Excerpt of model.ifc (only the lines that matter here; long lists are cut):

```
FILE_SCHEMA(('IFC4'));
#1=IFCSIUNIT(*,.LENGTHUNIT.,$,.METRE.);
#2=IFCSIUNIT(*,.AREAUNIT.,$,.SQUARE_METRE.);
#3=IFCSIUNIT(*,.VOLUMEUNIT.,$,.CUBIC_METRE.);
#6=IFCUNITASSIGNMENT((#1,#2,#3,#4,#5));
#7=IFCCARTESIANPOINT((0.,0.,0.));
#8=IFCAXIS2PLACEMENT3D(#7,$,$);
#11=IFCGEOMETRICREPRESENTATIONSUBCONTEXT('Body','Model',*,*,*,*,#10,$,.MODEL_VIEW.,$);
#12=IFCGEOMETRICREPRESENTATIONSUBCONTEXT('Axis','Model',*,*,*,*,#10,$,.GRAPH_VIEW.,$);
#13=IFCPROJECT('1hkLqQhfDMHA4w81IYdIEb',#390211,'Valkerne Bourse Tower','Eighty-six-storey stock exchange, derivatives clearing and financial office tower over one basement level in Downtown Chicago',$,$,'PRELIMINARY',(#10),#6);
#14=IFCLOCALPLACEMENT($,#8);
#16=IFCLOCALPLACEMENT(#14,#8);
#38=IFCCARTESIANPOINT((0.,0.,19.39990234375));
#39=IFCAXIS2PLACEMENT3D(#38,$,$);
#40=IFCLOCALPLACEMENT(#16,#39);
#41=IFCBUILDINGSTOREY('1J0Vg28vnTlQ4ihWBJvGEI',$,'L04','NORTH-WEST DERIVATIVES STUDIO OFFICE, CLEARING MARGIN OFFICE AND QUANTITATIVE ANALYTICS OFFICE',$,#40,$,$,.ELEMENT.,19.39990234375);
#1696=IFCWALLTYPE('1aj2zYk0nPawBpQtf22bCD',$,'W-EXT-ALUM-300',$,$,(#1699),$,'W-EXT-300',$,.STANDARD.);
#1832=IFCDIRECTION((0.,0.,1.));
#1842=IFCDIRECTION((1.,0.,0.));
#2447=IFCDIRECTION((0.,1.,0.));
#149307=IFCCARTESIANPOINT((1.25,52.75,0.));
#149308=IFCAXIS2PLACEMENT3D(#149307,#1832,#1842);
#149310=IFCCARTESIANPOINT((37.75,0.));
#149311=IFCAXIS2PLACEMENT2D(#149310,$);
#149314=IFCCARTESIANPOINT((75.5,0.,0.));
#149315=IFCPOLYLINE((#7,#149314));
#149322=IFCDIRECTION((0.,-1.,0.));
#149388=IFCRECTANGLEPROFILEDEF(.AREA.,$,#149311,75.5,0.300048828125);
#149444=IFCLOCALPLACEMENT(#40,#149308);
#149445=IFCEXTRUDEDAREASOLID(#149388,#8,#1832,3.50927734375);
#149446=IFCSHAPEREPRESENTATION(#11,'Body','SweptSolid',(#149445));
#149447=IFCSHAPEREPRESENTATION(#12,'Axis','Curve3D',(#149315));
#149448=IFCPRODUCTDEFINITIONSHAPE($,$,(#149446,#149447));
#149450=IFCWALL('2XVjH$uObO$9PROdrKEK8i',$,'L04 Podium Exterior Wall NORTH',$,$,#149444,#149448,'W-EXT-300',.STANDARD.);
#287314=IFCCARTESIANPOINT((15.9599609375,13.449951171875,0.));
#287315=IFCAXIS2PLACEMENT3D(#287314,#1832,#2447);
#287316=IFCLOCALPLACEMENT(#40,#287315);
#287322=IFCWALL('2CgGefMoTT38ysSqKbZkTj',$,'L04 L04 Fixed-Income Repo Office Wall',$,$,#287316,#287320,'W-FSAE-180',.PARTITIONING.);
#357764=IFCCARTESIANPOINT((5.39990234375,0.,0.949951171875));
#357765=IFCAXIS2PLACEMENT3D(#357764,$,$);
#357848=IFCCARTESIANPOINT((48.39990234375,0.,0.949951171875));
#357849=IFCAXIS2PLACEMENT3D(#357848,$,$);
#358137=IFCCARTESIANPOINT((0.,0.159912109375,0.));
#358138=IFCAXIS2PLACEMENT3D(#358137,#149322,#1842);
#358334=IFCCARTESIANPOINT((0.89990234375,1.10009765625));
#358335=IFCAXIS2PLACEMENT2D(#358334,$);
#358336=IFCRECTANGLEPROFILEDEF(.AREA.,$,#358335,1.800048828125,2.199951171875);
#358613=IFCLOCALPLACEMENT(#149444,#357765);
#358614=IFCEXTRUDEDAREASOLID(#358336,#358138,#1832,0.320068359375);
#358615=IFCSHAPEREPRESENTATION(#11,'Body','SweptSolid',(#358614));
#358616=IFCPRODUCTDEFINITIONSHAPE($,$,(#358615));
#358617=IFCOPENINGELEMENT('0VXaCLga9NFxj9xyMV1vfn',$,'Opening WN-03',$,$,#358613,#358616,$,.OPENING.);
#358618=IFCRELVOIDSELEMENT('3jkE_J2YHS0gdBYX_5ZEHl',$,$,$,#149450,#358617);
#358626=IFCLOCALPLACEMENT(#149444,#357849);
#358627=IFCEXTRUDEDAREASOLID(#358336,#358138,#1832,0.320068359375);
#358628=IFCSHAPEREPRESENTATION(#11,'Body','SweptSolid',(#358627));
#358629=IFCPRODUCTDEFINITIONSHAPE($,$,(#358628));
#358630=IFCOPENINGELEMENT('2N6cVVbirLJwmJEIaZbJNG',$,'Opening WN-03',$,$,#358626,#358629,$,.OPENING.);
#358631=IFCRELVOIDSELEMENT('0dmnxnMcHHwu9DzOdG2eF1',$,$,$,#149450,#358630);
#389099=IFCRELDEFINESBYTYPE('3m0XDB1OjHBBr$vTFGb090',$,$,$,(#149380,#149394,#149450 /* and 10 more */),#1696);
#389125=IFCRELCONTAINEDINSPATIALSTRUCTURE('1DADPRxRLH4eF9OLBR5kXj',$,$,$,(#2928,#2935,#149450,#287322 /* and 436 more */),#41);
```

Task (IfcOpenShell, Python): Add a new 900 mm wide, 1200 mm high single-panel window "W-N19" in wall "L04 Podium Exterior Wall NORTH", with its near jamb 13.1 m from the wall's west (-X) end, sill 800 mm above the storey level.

```python
import numpy as np
import ifcopenshell
import ifcopenshell.api.feature
import ifcopenshell.api.geometry
import ifcopenshell.api.root
import ifcopenshell.api.spatial
import ifcopenshell.geom
import ifcopenshell.util.element
import ifcopenshell.util.placement
import ifcopenshell.util.representation
import ifcopenshell.util.shape
import ifcopenshell.util.unit

model = ifcopenshell.open("model.ifc")
unit_scale = ifcopenshell.util.unit.calculate_unit_scale(model)
settings = ifcopenshell.geom.settings()


def volume(element):
    """Net volume in cubic metres, openings subtracted."""
    shape = ifcopenshell.geom.create_shape(settings, element)
    return ifcopenshell.util.shape.get_volume(shape.geometry)


wall = model.by_id(149450)
storey = ifcopenshell.util.element.get_container(wall, ifc_class="IfcBuildingStorey")
context = ifcopenshell.util.representation.get_context(model, "Model", "Body", "MODEL_VIEW")
before = volume(wall)

width, height, from_end, sill = 0.9, 1.2, 13.1, 0.8  # metres

# The wall runs along its own X axis, and the end named is its -X end.
wall_shape = ifcopenshell.geom.create_shape(settings, wall)
x, y, z = ifcopenshell.util.shape.get_vertices(wall_shape.geometry).T
start = x.min() + from_end
face, thickness = float(y.min()), float(y.max() - y.min())
wall_matrix = ifcopenshell.util.placement.get_local_placement(wall.ObjectPlacement)
level = ifcopenshell.util.placement.get_local_placement(storey.ObjectPlacement)[2, 3]


def in_wall(x, y):
    """Placement at x, y metres in the wall's axes, at sill height."""
    matrix = wall_matrix.copy()
    matrix[:, 3] = wall_matrix @ np.array([x / unit_scale, y / unit_scale, 0.0, 1.0])
    matrix[2, 3] = level + sill / unit_scale
    return matrix


# Opening: a box that overshoots both wall faces by 50 mm.
opening = ifcopenshell.api.root.create_entity(model, ifc_class="IfcOpeningElement", predefined_type="OPENING")
box = ifcopenshell.api.geometry.add_wall_representation(
    model, context=context, length=width, height=height, thickness=thickness + 0.1
)
ifcopenshell.api.geometry.assign_representation(model, product=opening, representation=box)
ifcopenshell.api.geometry.edit_object_placement(model, product=opening, matrix=in_wall(start, face - 0.05), is_si=False)
ifcopenshell.api.feature.add_feature(model, feature=opening, element=wall)

window = ifcopenshell.api.root.create_entity(model, ifc_class="IfcWindow", name="W-N19", predefined_type="WINDOW")
window.OverallWidth, window.OverallHeight = width / unit_scale, height / unit_scale
window.PartitioningType = "SINGLE_PANEL"
body = ifcopenshell.api.geometry.add_window_representation(
    model,
    context=context,
    overall_width=window.OverallWidth,
    overall_height=window.OverallHeight,
    partition_type="SINGLE_PANEL",
)
ifcopenshell.api.geometry.assign_representation(model, product=window, representation=body)
ifcopenshell.api.spatial.assign_container(model, products=[window], relating_structure=storey)
ifcopenshell.api.feature.add_filling(model, opening=opening, element=window)

# Centre the window in the wall's thickness.
ifcopenshell.api.geometry.edit_object_placement(model, product=window, matrix=in_wall(start, face), is_si=False)
window_shape = ifcopenshell.geom.create_shape(settings, window)
depth = ifcopenshell.util.shape.get_vertices(window_shape.geometry)[:, 1]
offset = face + thickness / 2 - (depth.min() + depth.max()) / 2
ifcopenshell.api.geometry.edit_object_placement(model, product=window, matrix=in_wall(start, offset), is_si=False)

after = volume(wall)

print(f"wall volume {before:.3f} -> {after:.3f} m3")

model.write("model-out.ifc")
```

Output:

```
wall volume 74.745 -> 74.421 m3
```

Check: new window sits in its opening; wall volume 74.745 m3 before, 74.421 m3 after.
